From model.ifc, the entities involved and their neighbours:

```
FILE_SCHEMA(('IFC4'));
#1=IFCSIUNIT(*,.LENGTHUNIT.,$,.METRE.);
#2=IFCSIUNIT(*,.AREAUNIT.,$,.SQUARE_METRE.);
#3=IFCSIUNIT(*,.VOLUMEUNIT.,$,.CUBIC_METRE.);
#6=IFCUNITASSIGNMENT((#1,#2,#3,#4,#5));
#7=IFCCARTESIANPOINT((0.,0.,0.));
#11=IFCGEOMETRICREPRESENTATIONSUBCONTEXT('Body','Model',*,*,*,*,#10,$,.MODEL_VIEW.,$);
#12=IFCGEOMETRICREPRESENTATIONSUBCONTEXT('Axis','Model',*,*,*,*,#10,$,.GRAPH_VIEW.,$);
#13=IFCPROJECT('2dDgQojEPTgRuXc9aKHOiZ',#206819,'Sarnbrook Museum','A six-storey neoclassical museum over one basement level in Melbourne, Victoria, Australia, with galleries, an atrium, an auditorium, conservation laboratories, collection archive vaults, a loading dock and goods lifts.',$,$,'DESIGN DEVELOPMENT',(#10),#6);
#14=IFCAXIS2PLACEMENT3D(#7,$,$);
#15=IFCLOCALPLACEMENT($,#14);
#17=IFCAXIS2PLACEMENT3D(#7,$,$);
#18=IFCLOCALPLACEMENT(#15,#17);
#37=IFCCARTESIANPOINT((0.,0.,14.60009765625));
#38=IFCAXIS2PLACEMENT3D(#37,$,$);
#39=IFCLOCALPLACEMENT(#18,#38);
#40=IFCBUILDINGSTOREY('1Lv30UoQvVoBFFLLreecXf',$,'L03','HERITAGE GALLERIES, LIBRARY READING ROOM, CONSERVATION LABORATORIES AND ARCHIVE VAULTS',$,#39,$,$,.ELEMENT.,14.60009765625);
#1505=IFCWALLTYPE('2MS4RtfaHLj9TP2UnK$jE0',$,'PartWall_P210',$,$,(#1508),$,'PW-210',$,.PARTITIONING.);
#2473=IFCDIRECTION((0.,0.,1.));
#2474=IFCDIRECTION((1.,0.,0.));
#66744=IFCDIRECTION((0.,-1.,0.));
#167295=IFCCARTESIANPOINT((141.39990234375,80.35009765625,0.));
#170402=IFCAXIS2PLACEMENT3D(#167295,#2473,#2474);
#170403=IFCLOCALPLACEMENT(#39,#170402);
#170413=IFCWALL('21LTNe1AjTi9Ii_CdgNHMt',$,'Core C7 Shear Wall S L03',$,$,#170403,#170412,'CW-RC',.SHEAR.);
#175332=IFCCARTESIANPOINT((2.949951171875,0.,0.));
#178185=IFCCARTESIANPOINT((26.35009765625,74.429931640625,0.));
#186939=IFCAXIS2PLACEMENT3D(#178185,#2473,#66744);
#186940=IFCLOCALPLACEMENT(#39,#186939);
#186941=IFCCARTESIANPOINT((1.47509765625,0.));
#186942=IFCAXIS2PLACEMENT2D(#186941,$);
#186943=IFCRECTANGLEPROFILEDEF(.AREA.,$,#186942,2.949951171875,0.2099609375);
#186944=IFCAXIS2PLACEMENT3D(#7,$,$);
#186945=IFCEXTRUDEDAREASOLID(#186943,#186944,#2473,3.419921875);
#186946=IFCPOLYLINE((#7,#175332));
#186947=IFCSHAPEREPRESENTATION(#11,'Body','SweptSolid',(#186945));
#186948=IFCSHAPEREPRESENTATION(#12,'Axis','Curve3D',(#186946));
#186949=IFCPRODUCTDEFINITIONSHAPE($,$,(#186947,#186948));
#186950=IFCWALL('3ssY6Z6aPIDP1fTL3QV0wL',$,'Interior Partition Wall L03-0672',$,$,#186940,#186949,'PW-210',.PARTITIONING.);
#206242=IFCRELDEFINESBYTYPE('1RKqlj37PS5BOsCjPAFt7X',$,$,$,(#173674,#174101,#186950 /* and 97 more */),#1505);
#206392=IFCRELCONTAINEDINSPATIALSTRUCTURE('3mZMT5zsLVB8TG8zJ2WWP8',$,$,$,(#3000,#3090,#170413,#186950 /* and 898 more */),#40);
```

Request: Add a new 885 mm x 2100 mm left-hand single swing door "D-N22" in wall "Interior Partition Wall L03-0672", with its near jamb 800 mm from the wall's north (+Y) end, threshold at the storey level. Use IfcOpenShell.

```python
import numpy as np
import ifcopenshell
import ifcopenshell.api.feature
import ifcopenshell.api.geometry
import ifcopenshell.api.root
import ifcopenshell.api.spatial
import ifcopenshell.geom
import ifcopenshell.util.element
import ifcopenshell.util.placement
import ifcopenshell.util.representation
import ifcopenshell.util.shape
import ifcopenshell.util.unit

model = ifcopenshell.open("model.ifc")
unit_scale = ifcopenshell.util.unit.calculate_unit_scale(model)
settings = ifcopenshell.geom.settings()


def volume(element):
    """Net volume in cubic metres, openings subtracted."""
    shape = ifcopenshell.geom.create_shape(settings, element)
    return ifcopenshell.util.shape.get_volume(shape.geometry)


wall = model.by_id(186950)
storey = ifcopenshell.util.element.get_container(wall, ifc_class="IfcBuildingStorey")
context = ifcopenshell.util.representation.get_context(model, "Model", "Body", "MODEL_VIEW")
before = volume(wall)

width, height, from_end, sill = 0.885, 2.1, 0.8, 0.0  # metres

# The wall runs along its own X axis, and the end named is its -X end.
wall_shape = ifcopenshell.geom.create_shape(settings, wall)
x, y, z = ifcopenshell.util.shape.get_vertices(wall_shape.geometry).T
start = x.min() + from_end
face, thickness = float(y.min()), float(y.max() - y.min())
wall_matrix = ifcopenshell.util.placement.get_local_placement(wall.ObjectPlacement)
level = ifcopenshell.util.placement.get_local_placement(storey.ObjectPlacement)[2, 3]


def in_wall(x, y):
    """Placement at x, y metres in the wall's axes, at sill height."""
    matrix = wall_matrix.copy()
    matrix[:, 3] = wall_matrix @ np.array([x / unit_scale, y / unit_scale, 0.0, 1.0])
    matrix[2, 3] = level + sill / unit_scale
    return matrix


# Opening: a box that overshoots both wall faces by 50 mm.
opening = ifcopenshell.api.root.create_entity(model, ifc_class="IfcOpeningElement", predefined_type="OPENING")
box = ifcopenshell.api.geometry.add_wall_representation(
    model, context=context, length=width, height=height, thickness=thickness + 0.1
)
ifcopenshell.api.geometry.assign_representation(model, product=opening, representation=box)
ifcopenshell.api.geometry.edit_object_placement(model, product=opening, matrix=in_wall(start, face - 0.05), is_si=False)
ifcopenshell.api.feature.add_feature(model, feature=opening, element=wall)

door = ifcopenshell.api.root.create_entity(model, ifc_class="IfcDoor", name="D-N22", predefined_type="DOOR")
door.OverallWidth, door.OverallHeight = width / unit_scale, height / unit_scale
door.OperationType = "SINGLE_SWING_LEFT"
body = ifcopenshell.api.geometry.add_door_representation(
    model,
    context=context,
    overall_width=door.OverallWidth,
    overall_height=door.OverallHeight,
    operation_type="SINGLE_SWING_LEFT",
    lining_properties={"LiningDepth": thickness / unit_scale, "ThresholdDepth": thickness / unit_scale},
)
ifcopenshell.api.geometry.assign_representation(model, product=door, representation=body)
ifcopenshell.api.spatial.assign_container(model, products=[door], relating_structure=storey)
ifcopenshell.api.feature.add_filling(model, opening=opening, element=door)

# The lining spans the wall, so the door starts at the wall face.
ifcopenshell.api.geometry.edit_object_placement(model, product=door, matrix=in_wall(start, face), is_si=False)

after = volume(wall)

print(f"wall volume {before:.3f} -> {after:.3f} m3")

model.write("model-out.ifc")
```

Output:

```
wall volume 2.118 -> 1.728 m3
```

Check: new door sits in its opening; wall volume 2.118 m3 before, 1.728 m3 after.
